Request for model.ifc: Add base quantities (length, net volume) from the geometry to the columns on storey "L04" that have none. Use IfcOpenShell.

First a look at what the model holds.

```python
import ifcopenshell
import ifcopenshell.util.element
import ifcopenshell.util.unit

model = ifcopenshell.open("model.ifc")
print(model.schema)
for unit_type in ("LENGTHUNIT", "AREAUNIT", "VOLUMEUNIT"):
    print(unit_type, ifcopenshell.util.unit.calculate_unit_scale(model, unit_type))
storey = next(s for s in model.by_type("IfcBuildingStorey") if s.Name == "L04")
columns = [e for e in ifcopenshell.util.element.get_decomposition(storey) if e.is_a("IfcColumn")]
for e in sorted(columns, key=lambda e: e.id()):
    print(e.id(), e.is_a(), e.Name, list(ifcopenshell.util.element.get_psets(e, qtos_only=True)), sep=" | ")
```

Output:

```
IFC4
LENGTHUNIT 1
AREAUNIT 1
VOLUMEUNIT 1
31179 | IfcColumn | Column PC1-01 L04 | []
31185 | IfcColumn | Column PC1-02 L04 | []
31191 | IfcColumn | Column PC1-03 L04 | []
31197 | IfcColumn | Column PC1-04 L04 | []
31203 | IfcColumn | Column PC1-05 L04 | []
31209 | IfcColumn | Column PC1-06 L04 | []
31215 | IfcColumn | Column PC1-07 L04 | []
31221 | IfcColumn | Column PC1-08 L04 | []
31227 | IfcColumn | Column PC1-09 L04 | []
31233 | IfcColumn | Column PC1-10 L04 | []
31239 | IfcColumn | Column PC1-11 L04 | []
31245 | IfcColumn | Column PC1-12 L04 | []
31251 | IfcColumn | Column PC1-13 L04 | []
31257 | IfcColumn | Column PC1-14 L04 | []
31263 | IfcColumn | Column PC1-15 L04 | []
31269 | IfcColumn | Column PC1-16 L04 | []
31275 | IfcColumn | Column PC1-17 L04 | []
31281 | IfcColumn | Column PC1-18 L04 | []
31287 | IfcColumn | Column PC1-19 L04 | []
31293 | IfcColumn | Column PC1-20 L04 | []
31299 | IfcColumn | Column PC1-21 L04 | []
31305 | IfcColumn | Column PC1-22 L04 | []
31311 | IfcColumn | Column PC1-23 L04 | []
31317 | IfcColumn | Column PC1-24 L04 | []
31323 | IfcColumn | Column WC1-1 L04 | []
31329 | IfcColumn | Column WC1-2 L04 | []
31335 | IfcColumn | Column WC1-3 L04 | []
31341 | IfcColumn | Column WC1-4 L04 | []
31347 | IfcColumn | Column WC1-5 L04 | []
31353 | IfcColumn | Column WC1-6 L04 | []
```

```python
import ifcopenshell
import ifcopenshell.api.pset
import ifcopenshell.geom
import ifcopenshell.util.element
import ifcopenshell.util.shape
import ifcopenshell.util.unit

model = ifcopenshell.open("model.ifc")
unit_scale = ifcopenshell.util.unit.calculate_unit_scale(model)
volume_scale = ifcopenshell.util.unit.calculate_unit_scale(model, "VOLUMEUNIT")
settings = ifcopenshell.geom.settings()

storey = next(s for s in model.by_type("IfcBuildingStorey") if s.Name == "L04")
columns = [e for e in ifcopenshell.util.element.get_decomposition(storey) if e.is_a("IfcColumn")]

for e in sorted(columns, key=lambda e: e.id()):
    if ifcopenshell.util.element.get_psets(e, qtos_only=True, should_inherit=False):
        continue
    # Geometry comes back in metres, in the element's own axes.
    shape = ifcopenshell.geom.create_shape(settings, e)
    values = {
        "Length": ifcopenshell.util.shape.get_z(shape.geometry) / unit_scale,
        "NetVolume": ifcopenshell.util.shape.get_volume(shape.geometry) / volume_scale,
    }
    qto = ifcopenshell.api.pset.add_qto(model, product=e, name="Qto_ColumnBaseQuantities")
    ifcopenshell.api.pset.edit_qto(model, qto=qto, properties=values)
    print(e.id(), {k: round(v, 3) for k, v in values.items()})

model.write("model_updated.ifc")
```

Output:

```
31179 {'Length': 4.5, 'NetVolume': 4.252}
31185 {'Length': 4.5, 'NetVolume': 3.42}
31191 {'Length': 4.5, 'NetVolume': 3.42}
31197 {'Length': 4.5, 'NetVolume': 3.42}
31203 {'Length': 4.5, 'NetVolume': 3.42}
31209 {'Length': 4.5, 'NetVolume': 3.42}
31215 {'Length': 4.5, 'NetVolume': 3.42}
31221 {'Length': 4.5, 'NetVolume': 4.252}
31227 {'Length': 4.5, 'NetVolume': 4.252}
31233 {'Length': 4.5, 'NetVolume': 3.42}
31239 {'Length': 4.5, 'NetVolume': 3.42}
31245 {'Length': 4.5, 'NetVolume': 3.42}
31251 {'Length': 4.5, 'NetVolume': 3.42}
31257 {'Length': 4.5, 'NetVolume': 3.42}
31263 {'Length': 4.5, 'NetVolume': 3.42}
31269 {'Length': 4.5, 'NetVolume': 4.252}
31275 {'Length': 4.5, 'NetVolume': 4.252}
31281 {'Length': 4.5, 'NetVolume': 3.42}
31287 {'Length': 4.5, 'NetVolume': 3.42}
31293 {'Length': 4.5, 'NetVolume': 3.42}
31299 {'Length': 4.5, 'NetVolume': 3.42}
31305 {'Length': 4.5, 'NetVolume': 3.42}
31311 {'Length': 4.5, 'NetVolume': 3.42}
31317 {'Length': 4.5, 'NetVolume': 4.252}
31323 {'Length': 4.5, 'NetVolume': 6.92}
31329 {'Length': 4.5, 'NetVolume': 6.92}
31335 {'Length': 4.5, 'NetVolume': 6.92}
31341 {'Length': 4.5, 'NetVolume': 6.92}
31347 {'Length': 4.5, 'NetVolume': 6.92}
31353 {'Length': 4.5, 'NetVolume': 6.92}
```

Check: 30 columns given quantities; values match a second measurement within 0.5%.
